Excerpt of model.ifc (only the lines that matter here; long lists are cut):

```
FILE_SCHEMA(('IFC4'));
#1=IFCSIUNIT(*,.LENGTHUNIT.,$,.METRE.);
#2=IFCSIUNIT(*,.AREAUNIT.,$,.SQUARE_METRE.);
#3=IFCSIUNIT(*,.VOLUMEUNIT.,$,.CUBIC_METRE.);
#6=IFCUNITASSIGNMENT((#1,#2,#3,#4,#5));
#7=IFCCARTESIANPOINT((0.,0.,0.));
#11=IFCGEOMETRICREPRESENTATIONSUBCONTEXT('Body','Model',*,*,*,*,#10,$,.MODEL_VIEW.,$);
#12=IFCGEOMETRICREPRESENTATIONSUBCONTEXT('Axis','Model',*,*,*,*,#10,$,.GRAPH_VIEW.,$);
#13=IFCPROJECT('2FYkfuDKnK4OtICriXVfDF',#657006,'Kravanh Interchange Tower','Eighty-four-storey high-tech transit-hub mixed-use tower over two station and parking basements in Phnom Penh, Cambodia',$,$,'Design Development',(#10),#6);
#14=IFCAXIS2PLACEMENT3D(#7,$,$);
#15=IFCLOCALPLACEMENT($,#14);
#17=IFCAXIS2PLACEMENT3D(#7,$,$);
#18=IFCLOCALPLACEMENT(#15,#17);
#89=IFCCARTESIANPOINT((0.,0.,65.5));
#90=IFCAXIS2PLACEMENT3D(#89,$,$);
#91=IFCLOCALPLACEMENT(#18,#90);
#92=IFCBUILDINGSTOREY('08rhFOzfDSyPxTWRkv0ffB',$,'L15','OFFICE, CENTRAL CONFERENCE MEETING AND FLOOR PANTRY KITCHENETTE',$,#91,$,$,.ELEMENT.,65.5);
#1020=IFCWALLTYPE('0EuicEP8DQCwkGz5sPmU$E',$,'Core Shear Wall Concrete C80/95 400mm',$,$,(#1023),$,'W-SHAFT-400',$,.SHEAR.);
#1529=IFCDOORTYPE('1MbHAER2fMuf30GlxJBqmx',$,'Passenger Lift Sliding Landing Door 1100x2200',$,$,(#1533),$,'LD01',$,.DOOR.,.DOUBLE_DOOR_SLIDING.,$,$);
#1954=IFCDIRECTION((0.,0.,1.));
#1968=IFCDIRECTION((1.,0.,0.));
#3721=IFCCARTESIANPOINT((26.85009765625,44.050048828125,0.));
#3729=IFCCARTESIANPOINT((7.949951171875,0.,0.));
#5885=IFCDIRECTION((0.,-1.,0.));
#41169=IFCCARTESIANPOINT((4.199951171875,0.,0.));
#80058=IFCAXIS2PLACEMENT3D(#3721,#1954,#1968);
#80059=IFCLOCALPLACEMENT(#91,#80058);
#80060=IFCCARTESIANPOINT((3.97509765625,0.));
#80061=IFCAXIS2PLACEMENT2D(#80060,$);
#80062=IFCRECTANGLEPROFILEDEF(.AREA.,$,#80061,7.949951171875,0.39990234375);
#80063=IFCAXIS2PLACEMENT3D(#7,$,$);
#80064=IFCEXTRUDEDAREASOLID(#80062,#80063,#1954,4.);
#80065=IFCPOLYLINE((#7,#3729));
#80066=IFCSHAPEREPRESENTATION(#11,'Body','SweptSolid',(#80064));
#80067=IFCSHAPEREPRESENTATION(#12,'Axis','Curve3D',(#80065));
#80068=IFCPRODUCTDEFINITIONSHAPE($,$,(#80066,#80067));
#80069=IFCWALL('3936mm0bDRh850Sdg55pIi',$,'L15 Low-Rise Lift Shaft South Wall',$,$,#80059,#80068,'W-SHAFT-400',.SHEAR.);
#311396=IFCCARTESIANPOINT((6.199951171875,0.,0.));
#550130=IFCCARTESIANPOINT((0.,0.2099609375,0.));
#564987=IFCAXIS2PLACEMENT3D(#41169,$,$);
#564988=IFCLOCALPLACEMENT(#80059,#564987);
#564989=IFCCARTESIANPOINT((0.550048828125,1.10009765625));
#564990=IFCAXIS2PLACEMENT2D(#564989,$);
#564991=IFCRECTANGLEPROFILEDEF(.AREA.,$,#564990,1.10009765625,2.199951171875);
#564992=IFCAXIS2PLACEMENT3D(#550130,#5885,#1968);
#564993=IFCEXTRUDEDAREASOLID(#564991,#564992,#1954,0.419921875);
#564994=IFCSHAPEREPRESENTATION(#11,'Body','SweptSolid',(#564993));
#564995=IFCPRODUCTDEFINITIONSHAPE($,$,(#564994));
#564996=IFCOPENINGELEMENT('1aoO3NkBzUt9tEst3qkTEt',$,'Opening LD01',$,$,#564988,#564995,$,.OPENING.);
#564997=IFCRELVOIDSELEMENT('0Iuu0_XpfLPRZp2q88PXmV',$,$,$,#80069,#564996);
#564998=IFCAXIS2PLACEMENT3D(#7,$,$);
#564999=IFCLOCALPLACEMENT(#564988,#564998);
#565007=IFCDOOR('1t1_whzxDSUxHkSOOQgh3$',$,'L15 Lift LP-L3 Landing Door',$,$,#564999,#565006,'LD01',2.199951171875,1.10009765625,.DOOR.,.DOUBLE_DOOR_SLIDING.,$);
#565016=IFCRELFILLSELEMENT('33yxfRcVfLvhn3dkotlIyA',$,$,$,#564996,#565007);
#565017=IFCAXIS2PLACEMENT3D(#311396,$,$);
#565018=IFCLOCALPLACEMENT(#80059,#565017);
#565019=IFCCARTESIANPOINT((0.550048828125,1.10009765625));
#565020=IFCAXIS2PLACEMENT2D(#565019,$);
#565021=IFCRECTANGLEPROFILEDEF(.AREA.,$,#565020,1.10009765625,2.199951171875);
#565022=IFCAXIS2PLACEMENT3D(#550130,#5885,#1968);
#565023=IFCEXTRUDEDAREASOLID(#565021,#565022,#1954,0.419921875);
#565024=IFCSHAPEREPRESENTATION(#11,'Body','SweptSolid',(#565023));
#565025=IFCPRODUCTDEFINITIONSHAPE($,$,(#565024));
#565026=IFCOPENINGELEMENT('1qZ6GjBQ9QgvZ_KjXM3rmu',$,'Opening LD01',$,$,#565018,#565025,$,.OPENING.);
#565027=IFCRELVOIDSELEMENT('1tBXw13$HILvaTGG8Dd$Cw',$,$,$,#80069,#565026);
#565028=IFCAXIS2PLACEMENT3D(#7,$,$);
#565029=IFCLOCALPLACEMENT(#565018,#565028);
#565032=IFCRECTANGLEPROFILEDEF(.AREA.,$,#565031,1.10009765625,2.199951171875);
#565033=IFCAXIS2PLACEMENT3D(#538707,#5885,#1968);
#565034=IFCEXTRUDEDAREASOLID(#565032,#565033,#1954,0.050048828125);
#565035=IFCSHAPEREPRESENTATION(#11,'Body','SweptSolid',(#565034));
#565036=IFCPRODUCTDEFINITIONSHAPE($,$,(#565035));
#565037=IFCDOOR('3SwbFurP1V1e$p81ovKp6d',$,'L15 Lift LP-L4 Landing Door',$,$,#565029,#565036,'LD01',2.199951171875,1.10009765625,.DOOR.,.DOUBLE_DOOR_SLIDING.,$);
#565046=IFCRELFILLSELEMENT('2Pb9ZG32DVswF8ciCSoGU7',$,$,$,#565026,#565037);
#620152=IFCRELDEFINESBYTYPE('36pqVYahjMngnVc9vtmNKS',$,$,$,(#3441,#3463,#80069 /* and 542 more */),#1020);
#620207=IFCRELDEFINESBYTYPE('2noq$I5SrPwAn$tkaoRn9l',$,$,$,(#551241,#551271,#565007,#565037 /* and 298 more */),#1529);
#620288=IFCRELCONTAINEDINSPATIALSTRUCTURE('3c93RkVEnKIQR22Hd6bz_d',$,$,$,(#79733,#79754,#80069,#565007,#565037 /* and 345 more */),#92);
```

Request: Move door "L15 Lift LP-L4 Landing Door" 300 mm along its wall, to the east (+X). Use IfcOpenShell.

```python
import ifcopenshell
import ifcopenshell.api.geometry
import ifcopenshell.util.placement

model = ifcopenshell.open("model.ifc")

door = model.by_guid("3SwbFurP1V1e$p81ovKp6d")
opening = door.FillsVoids[0].RelatingOpeningElement
wall = opening.VoidsElements[0].RelatingBuildingElement

wall_matrix = ifcopenshell.util.placement.get_local_placement(wall.ObjectPlacement)
shift = wall_matrix[:3, 0] * 0.3
before = ifcopenshell.util.placement.get_local_placement(door.ObjectPlacement)[:3, 3].copy()

# The door is placed relative to its opening, so it follows when the opening moves.
matrix = ifcopenshell.util.placement.get_local_placement(opening.ObjectPlacement)
matrix[:3, 3] += shift
ifcopenshell.api.geometry.edit_object_placement(
    model, product=opening, matrix=matrix, is_si=False, should_transform_children=True
)

after = ifcopenshell.util.placement.get_local_placement(door.ObjectPlacement)[:3, 3]
print("door moved by", (after - before).round(3) + 0.0)

model.write("model_updated.ifc")
```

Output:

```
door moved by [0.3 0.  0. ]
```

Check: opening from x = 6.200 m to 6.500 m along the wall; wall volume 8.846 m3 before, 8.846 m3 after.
